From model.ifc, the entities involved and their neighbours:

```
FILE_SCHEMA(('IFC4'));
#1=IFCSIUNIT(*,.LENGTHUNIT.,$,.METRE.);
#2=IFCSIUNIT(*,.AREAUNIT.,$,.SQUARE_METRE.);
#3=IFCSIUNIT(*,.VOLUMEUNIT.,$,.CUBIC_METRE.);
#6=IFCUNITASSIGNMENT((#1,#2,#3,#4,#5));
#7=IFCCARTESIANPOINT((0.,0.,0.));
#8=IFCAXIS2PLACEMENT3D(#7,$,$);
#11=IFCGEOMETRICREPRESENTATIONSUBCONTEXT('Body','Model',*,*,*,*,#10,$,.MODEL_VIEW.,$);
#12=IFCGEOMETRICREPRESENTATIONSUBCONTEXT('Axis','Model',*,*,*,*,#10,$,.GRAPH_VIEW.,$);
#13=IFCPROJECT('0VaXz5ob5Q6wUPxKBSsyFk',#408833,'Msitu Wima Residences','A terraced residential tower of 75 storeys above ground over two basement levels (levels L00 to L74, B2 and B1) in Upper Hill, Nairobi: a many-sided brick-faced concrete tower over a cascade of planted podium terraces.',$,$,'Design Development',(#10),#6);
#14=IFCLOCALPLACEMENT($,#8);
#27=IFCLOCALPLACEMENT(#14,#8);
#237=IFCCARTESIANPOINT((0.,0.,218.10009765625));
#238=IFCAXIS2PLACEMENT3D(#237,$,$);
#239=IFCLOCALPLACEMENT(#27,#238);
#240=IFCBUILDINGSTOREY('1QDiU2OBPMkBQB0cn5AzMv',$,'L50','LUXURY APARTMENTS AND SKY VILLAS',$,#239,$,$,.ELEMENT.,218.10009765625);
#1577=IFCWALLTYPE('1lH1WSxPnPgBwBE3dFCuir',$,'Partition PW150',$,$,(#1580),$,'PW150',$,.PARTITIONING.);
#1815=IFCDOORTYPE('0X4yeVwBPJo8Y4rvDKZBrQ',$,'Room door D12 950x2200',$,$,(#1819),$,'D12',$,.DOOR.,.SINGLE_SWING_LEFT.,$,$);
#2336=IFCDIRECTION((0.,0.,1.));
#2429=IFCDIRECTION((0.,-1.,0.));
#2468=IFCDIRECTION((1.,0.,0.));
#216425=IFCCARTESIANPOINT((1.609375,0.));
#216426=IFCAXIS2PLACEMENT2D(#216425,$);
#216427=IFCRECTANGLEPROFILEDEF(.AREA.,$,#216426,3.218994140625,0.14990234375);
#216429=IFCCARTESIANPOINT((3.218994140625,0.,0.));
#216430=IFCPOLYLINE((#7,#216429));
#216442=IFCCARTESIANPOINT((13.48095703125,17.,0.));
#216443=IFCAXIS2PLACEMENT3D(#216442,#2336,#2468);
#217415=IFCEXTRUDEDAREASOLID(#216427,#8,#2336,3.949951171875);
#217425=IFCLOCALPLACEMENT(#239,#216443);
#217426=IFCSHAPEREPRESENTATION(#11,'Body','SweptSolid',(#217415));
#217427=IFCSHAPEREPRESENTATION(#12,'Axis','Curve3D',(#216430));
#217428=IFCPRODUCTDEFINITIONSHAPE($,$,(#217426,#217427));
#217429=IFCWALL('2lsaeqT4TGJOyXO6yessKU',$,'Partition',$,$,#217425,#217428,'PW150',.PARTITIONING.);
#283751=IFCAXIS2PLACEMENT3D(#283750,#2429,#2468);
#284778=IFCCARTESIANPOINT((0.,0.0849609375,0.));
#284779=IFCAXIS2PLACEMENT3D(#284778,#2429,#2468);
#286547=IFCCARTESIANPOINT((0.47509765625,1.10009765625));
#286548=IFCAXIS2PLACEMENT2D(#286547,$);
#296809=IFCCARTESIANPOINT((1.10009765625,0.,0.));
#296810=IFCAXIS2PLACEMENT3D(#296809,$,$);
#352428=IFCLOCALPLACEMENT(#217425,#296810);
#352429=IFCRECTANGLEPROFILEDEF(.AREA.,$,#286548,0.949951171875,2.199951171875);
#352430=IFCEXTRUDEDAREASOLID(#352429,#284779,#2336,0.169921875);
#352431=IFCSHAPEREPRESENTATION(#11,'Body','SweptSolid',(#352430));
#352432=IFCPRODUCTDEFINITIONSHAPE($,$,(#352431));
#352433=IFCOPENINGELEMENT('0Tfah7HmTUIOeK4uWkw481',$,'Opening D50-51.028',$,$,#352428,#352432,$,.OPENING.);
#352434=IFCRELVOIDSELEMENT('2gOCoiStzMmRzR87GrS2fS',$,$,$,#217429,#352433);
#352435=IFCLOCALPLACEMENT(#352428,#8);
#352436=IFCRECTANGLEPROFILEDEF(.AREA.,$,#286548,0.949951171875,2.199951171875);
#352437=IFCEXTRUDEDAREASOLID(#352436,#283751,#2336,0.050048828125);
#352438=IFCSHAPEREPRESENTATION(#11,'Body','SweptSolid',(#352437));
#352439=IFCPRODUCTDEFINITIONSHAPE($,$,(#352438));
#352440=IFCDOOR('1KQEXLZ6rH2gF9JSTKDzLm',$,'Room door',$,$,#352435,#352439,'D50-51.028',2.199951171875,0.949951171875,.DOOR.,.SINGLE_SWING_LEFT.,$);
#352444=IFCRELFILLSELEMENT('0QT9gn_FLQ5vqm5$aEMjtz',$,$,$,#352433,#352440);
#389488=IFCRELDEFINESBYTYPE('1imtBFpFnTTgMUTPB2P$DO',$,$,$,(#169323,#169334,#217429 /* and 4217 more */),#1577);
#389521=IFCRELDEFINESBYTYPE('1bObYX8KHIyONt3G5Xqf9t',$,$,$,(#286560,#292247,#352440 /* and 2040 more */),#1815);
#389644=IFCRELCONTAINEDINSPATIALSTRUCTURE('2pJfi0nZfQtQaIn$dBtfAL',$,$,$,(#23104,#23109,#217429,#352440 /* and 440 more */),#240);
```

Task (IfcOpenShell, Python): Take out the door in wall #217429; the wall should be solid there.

```python
import ifcopenshell
import ifcopenshell.api.feature
import ifcopenshell.api.root
import ifcopenshell.geom
import ifcopenshell.util.shape

model = ifcopenshell.open("model.ifc")
settings = ifcopenshell.geom.settings()


def volume(element):
    """Net volume in cubic metres, openings subtracted."""
    shape = ifcopenshell.geom.create_shape(settings, element)
    return ifcopenshell.util.shape.get_volume(shape.geometry)


door = model.by_guid("1KQEXLZ6rH2gF9JSTKDzLm")
opening = door.FillsVoids[0].RelatingOpeningElement
wall = opening.VoidsElements[0].RelatingBuildingElement
before = volume(wall)

ifcopenshell.api.root.remove_product(model, product=door)
ifcopenshell.api.feature.remove_feature(model, feature=opening)

after = volume(wall)

print(f"wall volume {before:.3f} -> {after:.3f} m3")

model.write("model_edited.ifc")
```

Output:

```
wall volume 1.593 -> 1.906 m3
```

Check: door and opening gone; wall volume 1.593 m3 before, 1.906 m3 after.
